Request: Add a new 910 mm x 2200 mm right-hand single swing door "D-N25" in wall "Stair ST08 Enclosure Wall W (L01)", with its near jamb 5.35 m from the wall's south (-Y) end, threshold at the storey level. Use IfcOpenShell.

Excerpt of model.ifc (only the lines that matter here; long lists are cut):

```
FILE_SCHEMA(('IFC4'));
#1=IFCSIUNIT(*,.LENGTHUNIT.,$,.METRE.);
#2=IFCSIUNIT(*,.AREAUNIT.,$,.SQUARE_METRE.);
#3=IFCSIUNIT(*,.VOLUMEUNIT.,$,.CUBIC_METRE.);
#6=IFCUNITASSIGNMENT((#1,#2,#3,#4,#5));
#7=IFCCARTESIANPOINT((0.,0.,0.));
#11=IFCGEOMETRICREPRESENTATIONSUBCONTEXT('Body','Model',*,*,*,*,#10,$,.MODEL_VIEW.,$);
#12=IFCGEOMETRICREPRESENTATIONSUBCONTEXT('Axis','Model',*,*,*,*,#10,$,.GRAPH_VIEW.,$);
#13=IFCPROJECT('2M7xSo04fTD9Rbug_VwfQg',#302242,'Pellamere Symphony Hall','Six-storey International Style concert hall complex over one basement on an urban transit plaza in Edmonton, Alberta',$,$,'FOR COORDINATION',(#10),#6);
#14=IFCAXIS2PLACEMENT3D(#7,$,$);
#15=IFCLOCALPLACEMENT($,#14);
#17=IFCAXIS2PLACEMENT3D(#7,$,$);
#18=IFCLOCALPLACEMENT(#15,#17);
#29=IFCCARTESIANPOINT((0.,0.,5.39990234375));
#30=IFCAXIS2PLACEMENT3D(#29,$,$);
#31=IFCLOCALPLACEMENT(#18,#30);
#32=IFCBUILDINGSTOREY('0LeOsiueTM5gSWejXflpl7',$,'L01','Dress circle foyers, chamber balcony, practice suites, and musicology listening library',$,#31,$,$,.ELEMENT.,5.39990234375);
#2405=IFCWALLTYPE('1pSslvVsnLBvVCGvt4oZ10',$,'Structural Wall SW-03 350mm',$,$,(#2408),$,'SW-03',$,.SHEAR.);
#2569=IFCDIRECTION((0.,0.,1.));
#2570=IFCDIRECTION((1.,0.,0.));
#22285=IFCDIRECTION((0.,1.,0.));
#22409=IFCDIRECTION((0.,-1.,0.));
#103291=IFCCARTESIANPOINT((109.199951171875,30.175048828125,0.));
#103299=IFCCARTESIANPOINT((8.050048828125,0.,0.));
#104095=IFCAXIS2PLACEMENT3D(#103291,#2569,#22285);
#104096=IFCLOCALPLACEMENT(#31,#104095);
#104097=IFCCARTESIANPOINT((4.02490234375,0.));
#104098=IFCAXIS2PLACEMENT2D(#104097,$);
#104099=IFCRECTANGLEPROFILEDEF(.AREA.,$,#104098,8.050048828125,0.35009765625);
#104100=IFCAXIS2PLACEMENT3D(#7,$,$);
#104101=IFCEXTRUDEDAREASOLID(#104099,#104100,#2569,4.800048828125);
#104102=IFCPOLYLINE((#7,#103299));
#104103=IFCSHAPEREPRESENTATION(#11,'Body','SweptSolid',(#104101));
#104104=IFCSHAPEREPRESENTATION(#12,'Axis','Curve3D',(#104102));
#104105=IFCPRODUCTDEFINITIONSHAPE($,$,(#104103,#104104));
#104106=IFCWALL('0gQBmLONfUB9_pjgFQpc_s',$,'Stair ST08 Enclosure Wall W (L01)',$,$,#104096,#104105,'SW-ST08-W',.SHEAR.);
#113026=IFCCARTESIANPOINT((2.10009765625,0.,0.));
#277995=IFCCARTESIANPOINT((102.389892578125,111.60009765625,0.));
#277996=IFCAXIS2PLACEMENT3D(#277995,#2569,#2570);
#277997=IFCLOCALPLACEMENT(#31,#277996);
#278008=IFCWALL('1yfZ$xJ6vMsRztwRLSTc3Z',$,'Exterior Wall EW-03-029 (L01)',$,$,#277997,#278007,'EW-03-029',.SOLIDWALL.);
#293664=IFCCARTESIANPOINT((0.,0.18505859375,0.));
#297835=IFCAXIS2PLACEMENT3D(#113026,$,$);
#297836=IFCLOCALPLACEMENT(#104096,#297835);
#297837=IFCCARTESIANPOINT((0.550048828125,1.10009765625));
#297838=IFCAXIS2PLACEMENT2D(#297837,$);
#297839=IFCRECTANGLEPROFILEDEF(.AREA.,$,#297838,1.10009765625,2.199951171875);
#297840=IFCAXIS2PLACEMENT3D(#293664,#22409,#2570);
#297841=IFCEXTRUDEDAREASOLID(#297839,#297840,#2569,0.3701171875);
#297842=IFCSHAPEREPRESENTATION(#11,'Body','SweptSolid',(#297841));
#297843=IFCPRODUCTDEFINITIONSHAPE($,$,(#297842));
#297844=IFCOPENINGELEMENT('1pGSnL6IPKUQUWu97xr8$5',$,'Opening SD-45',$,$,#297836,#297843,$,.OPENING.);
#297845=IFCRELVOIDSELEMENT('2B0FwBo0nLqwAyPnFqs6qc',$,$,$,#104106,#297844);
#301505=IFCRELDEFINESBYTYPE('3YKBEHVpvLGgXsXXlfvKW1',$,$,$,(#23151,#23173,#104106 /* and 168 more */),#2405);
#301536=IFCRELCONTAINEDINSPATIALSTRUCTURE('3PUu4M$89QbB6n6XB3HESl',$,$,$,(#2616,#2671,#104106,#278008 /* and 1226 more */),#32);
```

```python
import numpy as np
import ifcopenshell
import ifcopenshell.api.feature
import ifcopenshell.api.geometry
import ifcopenshell.api.root
import ifcopenshell.api.spatial
import ifcopenshell.geom
import ifcopenshell.util.element
import ifcopenshell.util.placement
import ifcopenshell.util.representation
import ifcopenshell.util.shape
import ifcopenshell.util.unit

model = ifcopenshell.open("model.ifc")
unit_scale = ifcopenshell.util.unit.calculate_unit_scale(model)
settings = ifcopenshell.geom.settings()


def volume(element):
    """Net volume in cubic metres, openings subtracted."""
    shape = ifcopenshell.geom.create_shape(settings, element)
    return ifcopenshell.util.shape.get_volume(shape.geometry)


wall = model.by_guid("0gQBmLONfUB9_pjgFQpc_s")
storey = ifcopenshell.util.element.get_container(wall, ifc_class="IfcBuildingStorey")
context = ifcopenshell.util.representation.get_context(model, "Model", "Body", "MODEL_VIEW")
before = volume(wall)

width, height, from_end, sill = 0.91, 2.2, 5.35, 0.0  # metres

# The wall runs along its own X axis, and the end named is its -X end.
wall_shape = ifcopenshell.geom.create_shape(settings, wall)
x, y, z = ifcopenshell.util.shape.get_vertices(wall_shape.geometry).T
start = x.min() + from_end
face, thickness = float(y.min()), float(y.max() - y.min())
wall_matrix = ifcopenshell.util.placement.get_local_placement(wall.ObjectPlacement)
level = ifcopenshell.util.placement.get_local_placement(storey.ObjectPlacement)[2, 3]


def in_wall(x, y):
    """Placement at x, y metres in the wall's axes, at sill height."""
    matrix = wall_matrix.copy()
    matrix[:, 3] = wall_matrix @ np.array([x / unit_scale, y / unit_scale, 0.0, 1.0])
    matrix[2, 3] = level + sill / unit_scale
    return matrix


# Opening: a box that overshoots both wall faces by 50 mm.
opening = ifcopenshell.api.root.create_entity(model, ifc_class="IfcOpeningElement", predefined_type="OPENING")
box = ifcopenshell.api.geometry.add_wall_representation(
    model, context=context, length=width, height=height, thickness=thickness + 0.1
)
ifcopenshell.api.geometry.assign_representation(model, product=opening, representation=box)
ifcopenshell.api.geometry.edit_object_placement(model, product=opening, matrix=in_wall(start, face - 0.05), is_si=False)
ifcopenshell.api.feature.add_feature(model, feature=opening, element=wall)

door = ifcopenshell.api.root.create_entity(model, ifc_class="IfcDoor", name="D-N25", predefined_type="DOOR")
door.OverallWidth, door.OverallHeight = width / unit_scale, height / unit_scale
door.OperationType = "SINGLE_SWING_RIGHT"
body = ifcopenshell.api.geometry.add_door_representation(
    model,
    context=context,
    overall_width=door.OverallWidth,
    overall_height=door.OverallHeight,
    operation_type="SINGLE_SWING_RIGHT",
    lining_properties={"LiningDepth": thickness / unit_scale, "ThresholdDepth": thickness / unit_scale},
)
ifcopenshell.api.geometry.assign_representation(model, product=door, representation=body)
ifcopenshell.api.spatial.assign_container(model, products=[door], relating_structure=storey)
ifcopenshell.api.feature.add_filling(model, opening=opening, element=door)

# The lining spans the wall, so the door starts at the wall face.
ifcopenshell.api.geometry.edit_object_placement(model, product=door, matrix=in_wall(start, face), is_si=False)

after = volume(wall)

print(f"wall volume {before:.3f} -> {after:.3f} m3")

model.write("model-out.ifc")
```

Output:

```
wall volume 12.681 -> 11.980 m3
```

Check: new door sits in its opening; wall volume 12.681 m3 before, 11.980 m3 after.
